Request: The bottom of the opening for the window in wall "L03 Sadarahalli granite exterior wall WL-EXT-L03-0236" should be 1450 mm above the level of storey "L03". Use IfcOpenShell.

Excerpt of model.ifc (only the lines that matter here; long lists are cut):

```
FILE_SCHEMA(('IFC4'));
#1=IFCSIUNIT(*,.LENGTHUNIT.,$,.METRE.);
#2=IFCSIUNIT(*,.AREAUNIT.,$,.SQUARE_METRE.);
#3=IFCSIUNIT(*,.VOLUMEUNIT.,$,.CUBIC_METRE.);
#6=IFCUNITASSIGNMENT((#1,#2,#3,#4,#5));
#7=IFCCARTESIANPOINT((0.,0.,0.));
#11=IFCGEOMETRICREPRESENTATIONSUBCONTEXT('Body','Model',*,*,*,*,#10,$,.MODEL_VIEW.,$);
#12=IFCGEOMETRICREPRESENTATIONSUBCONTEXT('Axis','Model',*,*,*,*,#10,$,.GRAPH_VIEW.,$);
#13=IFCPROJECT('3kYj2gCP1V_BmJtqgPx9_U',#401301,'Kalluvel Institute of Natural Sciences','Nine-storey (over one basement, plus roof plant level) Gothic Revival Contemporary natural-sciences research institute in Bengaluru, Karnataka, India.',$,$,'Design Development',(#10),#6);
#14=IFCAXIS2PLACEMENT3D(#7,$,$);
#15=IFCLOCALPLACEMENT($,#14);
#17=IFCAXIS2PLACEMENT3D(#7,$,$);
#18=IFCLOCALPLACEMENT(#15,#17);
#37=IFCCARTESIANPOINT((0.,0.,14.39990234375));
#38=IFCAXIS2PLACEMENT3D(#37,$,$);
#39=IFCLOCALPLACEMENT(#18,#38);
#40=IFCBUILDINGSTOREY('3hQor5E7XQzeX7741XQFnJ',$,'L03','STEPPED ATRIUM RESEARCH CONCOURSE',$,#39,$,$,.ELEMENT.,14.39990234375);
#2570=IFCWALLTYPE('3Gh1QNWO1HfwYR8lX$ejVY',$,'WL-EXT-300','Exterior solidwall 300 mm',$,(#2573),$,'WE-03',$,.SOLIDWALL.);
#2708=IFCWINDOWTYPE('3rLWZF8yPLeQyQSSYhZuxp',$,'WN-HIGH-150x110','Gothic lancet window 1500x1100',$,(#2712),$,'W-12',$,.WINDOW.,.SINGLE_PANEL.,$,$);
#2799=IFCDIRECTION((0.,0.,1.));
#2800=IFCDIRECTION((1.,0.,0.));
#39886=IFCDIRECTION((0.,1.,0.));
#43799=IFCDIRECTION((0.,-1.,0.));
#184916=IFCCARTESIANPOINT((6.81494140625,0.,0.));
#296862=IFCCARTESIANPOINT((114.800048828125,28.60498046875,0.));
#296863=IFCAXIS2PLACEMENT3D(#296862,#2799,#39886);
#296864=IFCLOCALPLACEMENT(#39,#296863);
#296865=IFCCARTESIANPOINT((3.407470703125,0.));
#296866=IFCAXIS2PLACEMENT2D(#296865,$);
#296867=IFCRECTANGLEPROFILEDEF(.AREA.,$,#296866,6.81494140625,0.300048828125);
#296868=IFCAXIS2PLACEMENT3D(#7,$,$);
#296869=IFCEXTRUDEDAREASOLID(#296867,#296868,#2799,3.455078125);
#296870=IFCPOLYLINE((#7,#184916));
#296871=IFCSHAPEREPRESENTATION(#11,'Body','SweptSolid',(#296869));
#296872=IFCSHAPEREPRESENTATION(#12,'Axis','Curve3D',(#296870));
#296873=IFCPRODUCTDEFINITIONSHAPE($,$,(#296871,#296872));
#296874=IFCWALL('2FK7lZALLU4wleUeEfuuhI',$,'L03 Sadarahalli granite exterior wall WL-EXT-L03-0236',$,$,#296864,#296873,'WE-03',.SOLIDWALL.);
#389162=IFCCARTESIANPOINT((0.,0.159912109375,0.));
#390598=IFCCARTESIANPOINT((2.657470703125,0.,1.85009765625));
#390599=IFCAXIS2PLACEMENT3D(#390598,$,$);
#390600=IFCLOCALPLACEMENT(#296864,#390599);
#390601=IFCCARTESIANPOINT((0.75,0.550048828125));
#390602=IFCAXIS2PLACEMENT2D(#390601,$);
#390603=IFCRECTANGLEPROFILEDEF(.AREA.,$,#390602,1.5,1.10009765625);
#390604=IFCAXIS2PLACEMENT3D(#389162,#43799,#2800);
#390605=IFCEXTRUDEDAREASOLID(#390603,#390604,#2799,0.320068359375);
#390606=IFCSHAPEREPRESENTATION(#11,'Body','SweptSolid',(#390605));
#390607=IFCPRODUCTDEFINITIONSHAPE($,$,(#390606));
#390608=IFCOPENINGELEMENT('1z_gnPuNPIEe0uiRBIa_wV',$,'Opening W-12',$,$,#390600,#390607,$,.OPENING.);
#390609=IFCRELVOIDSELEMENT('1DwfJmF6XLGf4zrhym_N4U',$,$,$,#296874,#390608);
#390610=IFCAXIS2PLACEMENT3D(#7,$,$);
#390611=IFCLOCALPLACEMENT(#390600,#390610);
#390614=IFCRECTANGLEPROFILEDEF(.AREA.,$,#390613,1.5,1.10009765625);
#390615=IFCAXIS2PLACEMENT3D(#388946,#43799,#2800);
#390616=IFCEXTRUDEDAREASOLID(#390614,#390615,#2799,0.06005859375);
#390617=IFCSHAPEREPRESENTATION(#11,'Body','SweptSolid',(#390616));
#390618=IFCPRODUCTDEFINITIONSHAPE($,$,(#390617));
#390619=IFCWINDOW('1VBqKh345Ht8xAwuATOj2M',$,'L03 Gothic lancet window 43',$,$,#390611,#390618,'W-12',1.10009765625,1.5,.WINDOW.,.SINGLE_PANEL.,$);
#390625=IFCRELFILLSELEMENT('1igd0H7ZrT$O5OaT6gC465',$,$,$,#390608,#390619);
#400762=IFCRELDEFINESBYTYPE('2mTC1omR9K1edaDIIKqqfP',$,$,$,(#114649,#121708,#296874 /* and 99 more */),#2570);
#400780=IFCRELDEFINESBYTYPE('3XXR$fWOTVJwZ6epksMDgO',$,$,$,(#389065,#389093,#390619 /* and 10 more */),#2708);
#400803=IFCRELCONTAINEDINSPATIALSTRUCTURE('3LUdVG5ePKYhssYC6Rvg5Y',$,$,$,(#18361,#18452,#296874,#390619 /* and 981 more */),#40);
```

```python
import numpy as np
import ifcopenshell
import ifcopenshell.api.geometry
import ifcopenshell.geom
import ifcopenshell.util.element
import ifcopenshell.util.placement
import ifcopenshell.util.shape
import ifcopenshell.util.unit

model = ifcopenshell.open("model.ifc")
unit_scale = ifcopenshell.util.unit.calculate_unit_scale(model)

window = model.by_guid("1VBqKh345Ht8xAwuATOj2M")
opening = window.FillsVoids[0].RelatingOpeningElement
storey = ifcopenshell.util.element.get_container(window, ifc_class="IfcBuildingStorey")
level = ifcopenshell.util.placement.get_local_placement(storey.ObjectPlacement)[2, 3]

# The opening's origin need not be at the sill, so measure its lowest point.
shape = ifcopenshell.geom.create_shape(ifcopenshell.geom.settings(), opening)
bottom = ifcopenshell.util.shape.get_shape_bottom_elevation(shape, shape.geometry) / unit_scale
dz = level + 1.45 - bottom

shift = np.array([0.0, 0.0, dz])
# The window is placed relative to its opening, so it follows when the opening moves.
matrix = ifcopenshell.util.placement.get_local_placement(opening.ObjectPlacement)
matrix[:3, 3] += shift
ifcopenshell.api.geometry.edit_object_placement(
    model, product=opening, matrix=matrix, is_si=False, should_transform_children=True
)

print(f"moved by {dz * unit_scale:+.3f} m")

model.write("model_updated.ifc")
```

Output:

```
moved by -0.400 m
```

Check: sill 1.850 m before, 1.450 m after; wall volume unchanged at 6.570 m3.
